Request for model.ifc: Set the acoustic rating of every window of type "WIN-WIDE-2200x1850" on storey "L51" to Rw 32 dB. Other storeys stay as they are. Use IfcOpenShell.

First a look at what the model holds.

```python
import ifcopenshell
import ifcopenshell.util.element

model = ifcopenshell.open("model.ifc")
print(model.schema)
storey = next(s for s in model.by_type("IfcBuildingStorey") if s.Name == "L51")
windows = [e for e in ifcopenshell.util.element.get_decomposition(storey) if e.is_a("IfcWindow")]
seen = {}
for e in windows:
    element_type = ifcopenshell.util.element.get_type(e)
    key = (element_type.Name if element_type != e and element_type else None, ifcopenshell.util.element.get_pset(e, "Pset_WindowCommon", "AcousticRating"))
    seen[key] = seen.get(key, 0) + 1
for (name, value), count in sorted(seen.items(), key=str):
    print(count, "x", name, "|", value)
```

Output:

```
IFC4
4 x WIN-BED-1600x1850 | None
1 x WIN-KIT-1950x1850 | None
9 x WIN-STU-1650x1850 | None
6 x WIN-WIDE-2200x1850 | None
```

```python
import ifcopenshell
import ifcopenshell.api.pset
import ifcopenshell.util.element

model = ifcopenshell.open("model.ifc")

storey = next(s for s in model.by_type("IfcBuildingStorey") if s.Name == "L51")
windows = [e for e in ifcopenshell.util.element.get_decomposition(storey) if e.is_a("IfcWindow")]

count = 0
for e in windows:
    element_type = ifcopenshell.util.element.get_type(e)
    if element_type in (None, e) or element_type.Name != "WIN-WIDE-2200x1850":
        continue
    # add_pset returns the element's existing set when there is one.
    pset = ifcopenshell.api.pset.add_pset(model, product=e, name="Pset_WindowCommon")
    ifcopenshell.api.pset.edit_pset(model, pset=pset, properties={"AcousticRating": "Rw 32 dB"})
    count += 1

print(count, "windows updated")

model.write("model_v2.ifc")
```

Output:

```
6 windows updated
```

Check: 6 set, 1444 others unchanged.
